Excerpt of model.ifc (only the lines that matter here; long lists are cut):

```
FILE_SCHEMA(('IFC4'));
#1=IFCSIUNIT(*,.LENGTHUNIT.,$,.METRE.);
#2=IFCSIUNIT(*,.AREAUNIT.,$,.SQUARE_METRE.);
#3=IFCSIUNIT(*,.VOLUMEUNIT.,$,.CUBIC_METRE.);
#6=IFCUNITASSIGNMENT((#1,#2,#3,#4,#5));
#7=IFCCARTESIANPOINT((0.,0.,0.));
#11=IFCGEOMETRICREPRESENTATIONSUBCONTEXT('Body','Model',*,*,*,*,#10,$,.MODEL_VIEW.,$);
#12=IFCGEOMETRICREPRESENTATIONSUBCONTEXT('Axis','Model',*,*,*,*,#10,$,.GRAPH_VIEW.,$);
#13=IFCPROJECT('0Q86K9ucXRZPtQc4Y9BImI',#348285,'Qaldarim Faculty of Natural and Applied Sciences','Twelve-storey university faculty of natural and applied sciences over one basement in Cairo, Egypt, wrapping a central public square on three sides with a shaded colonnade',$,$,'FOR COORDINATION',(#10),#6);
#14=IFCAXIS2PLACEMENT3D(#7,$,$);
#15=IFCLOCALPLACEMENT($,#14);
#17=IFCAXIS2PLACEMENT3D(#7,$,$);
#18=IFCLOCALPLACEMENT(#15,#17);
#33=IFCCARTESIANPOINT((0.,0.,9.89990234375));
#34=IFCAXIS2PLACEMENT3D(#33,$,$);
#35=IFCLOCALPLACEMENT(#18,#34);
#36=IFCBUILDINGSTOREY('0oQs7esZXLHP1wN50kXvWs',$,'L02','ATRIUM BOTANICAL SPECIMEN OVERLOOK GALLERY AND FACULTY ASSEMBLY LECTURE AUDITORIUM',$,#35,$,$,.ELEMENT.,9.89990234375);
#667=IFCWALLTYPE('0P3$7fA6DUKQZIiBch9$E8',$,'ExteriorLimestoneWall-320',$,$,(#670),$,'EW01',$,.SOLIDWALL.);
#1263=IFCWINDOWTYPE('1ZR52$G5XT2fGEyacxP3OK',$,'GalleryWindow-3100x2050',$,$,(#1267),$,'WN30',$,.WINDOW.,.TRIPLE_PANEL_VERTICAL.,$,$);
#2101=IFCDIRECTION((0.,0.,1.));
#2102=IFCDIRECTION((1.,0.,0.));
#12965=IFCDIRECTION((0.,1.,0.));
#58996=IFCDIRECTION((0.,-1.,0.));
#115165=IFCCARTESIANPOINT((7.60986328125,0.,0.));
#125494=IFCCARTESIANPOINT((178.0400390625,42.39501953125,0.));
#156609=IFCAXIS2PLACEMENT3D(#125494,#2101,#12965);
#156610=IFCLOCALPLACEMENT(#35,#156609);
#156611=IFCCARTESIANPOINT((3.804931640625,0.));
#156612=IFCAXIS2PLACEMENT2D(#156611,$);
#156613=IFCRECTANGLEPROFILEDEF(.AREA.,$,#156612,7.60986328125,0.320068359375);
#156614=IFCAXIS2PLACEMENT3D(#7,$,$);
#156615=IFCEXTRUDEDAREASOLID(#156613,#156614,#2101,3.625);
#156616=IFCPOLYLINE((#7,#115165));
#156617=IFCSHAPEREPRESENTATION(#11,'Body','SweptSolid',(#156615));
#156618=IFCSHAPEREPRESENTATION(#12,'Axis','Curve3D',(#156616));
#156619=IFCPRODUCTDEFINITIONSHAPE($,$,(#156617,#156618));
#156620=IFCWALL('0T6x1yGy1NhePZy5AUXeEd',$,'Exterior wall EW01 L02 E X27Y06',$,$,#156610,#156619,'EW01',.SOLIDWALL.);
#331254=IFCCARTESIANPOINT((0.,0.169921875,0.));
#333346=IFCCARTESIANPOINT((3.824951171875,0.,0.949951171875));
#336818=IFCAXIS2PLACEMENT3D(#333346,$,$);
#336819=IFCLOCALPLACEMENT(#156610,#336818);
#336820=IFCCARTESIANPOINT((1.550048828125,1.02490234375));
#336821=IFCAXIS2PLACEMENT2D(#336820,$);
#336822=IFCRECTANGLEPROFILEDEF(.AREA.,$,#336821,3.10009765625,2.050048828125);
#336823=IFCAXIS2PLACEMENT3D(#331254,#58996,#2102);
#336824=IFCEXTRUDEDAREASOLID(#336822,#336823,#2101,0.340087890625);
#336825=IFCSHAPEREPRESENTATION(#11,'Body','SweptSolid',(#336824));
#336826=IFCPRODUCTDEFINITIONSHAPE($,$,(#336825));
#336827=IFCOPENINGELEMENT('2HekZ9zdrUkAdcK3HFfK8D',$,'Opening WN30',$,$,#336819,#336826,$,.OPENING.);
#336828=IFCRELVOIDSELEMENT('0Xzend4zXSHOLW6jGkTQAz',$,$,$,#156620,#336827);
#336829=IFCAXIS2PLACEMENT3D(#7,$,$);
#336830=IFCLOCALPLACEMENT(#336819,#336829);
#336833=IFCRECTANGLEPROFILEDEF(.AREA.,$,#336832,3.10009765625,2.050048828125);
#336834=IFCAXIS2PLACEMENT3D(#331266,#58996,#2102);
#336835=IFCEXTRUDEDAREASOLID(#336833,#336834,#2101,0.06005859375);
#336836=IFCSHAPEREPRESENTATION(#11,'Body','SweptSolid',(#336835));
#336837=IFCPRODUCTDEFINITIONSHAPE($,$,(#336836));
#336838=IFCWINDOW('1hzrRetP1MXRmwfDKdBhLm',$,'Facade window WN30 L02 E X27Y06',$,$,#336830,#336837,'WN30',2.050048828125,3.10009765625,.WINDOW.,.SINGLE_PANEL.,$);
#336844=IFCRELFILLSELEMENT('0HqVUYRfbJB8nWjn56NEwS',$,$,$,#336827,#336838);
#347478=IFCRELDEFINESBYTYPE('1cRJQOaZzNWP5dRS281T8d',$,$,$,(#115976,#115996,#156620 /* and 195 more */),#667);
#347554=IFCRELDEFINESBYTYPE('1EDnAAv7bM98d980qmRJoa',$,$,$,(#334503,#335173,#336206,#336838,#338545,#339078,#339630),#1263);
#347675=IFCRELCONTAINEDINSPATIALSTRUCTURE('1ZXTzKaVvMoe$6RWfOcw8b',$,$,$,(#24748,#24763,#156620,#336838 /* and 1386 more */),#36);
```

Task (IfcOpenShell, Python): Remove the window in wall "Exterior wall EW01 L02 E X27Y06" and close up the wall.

```python
import ifcopenshell
import ifcopenshell.api.feature
import ifcopenshell.api.root
import ifcopenshell.geom
import ifcopenshell.util.shape

model = ifcopenshell.open("model.ifc")
settings = ifcopenshell.geom.settings()


def volume(element):
    """Net volume in cubic metres, openings subtracted."""
    shape = ifcopenshell.geom.create_shape(settings, element)
    return ifcopenshell.util.shape.get_volume(shape.geometry)


window = model.by_guid("1hzrRetP1MXRmwfDKdBhLm")
opening = window.FillsVoids[0].RelatingOpeningElement
wall = opening.VoidsElements[0].RelatingBuildingElement
before = volume(wall)

ifcopenshell.api.root.remove_product(model, product=window)
ifcopenshell.api.feature.remove_feature(model, feature=opening)

after = volume(wall)

print(f"wall volume {before:.3f} -> {after:.3f} m3")

model.write("model_rev.ifc")
```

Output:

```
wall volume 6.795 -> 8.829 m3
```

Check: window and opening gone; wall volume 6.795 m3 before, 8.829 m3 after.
